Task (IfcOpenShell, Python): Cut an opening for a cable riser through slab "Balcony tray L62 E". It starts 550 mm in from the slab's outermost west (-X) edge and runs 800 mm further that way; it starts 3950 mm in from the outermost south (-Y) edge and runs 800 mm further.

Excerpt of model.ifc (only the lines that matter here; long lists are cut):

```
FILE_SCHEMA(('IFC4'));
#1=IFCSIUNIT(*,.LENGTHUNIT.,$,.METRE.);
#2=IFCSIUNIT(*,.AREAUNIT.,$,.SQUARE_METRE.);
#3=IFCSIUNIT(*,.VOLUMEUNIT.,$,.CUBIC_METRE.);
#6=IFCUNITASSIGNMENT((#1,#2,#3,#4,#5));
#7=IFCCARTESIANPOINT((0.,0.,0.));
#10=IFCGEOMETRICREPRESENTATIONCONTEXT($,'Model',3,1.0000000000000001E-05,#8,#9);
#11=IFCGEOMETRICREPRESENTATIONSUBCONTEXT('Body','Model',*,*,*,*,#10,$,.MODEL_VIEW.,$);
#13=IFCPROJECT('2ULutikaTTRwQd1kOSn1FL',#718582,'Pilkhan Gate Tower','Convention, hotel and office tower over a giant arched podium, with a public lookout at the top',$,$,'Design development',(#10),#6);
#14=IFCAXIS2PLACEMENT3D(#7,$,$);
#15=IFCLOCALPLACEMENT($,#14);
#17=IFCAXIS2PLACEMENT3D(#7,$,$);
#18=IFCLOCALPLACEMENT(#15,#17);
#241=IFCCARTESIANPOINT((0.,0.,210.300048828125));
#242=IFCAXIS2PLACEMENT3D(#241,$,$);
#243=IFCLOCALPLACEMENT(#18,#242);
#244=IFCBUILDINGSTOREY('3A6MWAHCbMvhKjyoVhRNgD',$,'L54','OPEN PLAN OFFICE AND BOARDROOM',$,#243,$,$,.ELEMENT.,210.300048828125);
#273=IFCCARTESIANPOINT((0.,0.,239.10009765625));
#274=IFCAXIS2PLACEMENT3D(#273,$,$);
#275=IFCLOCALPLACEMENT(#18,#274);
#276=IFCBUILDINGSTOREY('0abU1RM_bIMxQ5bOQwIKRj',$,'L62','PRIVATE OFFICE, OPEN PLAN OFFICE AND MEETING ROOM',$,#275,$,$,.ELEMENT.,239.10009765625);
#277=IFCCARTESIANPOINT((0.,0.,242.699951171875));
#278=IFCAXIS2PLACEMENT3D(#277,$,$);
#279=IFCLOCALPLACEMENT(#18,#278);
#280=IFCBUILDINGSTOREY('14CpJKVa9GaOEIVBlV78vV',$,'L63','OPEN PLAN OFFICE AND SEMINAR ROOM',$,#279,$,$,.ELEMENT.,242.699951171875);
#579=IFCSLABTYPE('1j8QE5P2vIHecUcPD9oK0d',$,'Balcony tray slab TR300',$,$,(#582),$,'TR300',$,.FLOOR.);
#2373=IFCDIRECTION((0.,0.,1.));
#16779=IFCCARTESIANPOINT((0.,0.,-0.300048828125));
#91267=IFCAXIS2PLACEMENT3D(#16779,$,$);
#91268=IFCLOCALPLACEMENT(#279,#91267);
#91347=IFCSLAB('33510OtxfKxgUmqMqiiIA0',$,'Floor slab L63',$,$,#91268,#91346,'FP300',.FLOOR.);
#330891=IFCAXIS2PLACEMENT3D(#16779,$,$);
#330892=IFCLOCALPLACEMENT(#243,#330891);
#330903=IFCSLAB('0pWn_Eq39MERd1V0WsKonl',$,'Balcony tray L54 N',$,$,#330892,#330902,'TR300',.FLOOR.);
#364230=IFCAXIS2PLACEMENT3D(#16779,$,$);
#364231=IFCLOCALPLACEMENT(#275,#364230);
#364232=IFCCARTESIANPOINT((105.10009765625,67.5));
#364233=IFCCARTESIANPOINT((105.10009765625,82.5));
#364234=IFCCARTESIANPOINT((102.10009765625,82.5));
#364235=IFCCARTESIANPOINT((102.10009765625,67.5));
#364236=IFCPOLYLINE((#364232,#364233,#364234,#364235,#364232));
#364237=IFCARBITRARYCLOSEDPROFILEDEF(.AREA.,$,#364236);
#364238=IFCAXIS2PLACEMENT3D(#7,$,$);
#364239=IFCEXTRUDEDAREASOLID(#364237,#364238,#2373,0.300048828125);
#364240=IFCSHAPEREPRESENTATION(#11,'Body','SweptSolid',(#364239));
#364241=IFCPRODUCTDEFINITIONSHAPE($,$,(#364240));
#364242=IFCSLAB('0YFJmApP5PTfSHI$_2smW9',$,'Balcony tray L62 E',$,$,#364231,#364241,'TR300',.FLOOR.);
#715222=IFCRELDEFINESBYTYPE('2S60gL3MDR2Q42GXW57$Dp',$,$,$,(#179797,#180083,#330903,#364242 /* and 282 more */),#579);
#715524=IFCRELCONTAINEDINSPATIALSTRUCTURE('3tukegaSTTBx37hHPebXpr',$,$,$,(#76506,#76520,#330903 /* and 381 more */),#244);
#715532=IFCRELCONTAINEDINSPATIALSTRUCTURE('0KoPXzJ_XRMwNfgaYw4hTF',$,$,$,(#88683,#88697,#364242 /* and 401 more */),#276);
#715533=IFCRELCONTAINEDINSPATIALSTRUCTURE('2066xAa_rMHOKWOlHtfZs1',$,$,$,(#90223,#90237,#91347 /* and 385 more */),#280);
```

```python
import numpy as np
import ifcopenshell
import ifcopenshell.api.feature
import ifcopenshell.api.geometry
import ifcopenshell.api.root
import ifcopenshell.geom
import ifcopenshell.util.placement
import ifcopenshell.util.representation
import ifcopenshell.util.shape
import ifcopenshell.util.unit

model = ifcopenshell.open("model.ifc")
unit_scale = ifcopenshell.util.unit.calculate_unit_scale(model)
settings = ifcopenshell.geom.settings()


def volume(element):
    """Net volume in cubic metres, openings subtracted."""
    shape = ifcopenshell.geom.create_shape(settings, element)
    return ifcopenshell.util.shape.get_volume(shape.geometry)


slab = model.by_guid("0YFJmApP5PTfSHI$_2smW9")
before = volume(slab)

# Extent in the slab's own axes, in metres. The edges named are its -X and -Y sides.
slab_shape = ifcopenshell.geom.create_shape(settings, slab)
vertices = ifcopenshell.util.shape.get_vertices(slab_shape.geometry)
x_min, y_min, bottom = vertices.min(axis=0)
top = vertices[:, 2].max()

opening = ifcopenshell.api.root.create_entity(model, ifc_class="IfcOpeningElement", name="Cable riser opening", predefined_type="OPENING")
context = ifcopenshell.util.representation.get_context(model, "Model", "Body", "MODEL_VIEW")
width, depth = 0.8, 0.8
outline = [(0.0, 0.0), (width, 0.0), (width, depth), (0.0, depth), (0.0, 0.0)]
# Overshoot both faces by 50 mm so the cut is clean.
shape = ifcopenshell.api.geometry.add_slab_representation(
    model, context=context, depth=top - bottom + 0.1, polyline=outline
)
ifcopenshell.api.geometry.assign_representation(model, product=opening, representation=shape)

matrix = ifcopenshell.util.placement.get_local_placement(slab.ObjectPlacement)
matrix[:, 3] = matrix @ np.append(np.array([x_min + 0.55, y_min + 3.95, bottom - 0.05]) / unit_scale, 1.0)
ifcopenshell.api.geometry.edit_object_placement(model, product=opening, matrix=matrix, is_si=False)
ifcopenshell.api.feature.add_feature(model, feature=opening, element=slab)

after = volume(slab)

print(f"slab volume {before:.3f} -> {after:.3f} m3")

model.write("model-out.ifc")
```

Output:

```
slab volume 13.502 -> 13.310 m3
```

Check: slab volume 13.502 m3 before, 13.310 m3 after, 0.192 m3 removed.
